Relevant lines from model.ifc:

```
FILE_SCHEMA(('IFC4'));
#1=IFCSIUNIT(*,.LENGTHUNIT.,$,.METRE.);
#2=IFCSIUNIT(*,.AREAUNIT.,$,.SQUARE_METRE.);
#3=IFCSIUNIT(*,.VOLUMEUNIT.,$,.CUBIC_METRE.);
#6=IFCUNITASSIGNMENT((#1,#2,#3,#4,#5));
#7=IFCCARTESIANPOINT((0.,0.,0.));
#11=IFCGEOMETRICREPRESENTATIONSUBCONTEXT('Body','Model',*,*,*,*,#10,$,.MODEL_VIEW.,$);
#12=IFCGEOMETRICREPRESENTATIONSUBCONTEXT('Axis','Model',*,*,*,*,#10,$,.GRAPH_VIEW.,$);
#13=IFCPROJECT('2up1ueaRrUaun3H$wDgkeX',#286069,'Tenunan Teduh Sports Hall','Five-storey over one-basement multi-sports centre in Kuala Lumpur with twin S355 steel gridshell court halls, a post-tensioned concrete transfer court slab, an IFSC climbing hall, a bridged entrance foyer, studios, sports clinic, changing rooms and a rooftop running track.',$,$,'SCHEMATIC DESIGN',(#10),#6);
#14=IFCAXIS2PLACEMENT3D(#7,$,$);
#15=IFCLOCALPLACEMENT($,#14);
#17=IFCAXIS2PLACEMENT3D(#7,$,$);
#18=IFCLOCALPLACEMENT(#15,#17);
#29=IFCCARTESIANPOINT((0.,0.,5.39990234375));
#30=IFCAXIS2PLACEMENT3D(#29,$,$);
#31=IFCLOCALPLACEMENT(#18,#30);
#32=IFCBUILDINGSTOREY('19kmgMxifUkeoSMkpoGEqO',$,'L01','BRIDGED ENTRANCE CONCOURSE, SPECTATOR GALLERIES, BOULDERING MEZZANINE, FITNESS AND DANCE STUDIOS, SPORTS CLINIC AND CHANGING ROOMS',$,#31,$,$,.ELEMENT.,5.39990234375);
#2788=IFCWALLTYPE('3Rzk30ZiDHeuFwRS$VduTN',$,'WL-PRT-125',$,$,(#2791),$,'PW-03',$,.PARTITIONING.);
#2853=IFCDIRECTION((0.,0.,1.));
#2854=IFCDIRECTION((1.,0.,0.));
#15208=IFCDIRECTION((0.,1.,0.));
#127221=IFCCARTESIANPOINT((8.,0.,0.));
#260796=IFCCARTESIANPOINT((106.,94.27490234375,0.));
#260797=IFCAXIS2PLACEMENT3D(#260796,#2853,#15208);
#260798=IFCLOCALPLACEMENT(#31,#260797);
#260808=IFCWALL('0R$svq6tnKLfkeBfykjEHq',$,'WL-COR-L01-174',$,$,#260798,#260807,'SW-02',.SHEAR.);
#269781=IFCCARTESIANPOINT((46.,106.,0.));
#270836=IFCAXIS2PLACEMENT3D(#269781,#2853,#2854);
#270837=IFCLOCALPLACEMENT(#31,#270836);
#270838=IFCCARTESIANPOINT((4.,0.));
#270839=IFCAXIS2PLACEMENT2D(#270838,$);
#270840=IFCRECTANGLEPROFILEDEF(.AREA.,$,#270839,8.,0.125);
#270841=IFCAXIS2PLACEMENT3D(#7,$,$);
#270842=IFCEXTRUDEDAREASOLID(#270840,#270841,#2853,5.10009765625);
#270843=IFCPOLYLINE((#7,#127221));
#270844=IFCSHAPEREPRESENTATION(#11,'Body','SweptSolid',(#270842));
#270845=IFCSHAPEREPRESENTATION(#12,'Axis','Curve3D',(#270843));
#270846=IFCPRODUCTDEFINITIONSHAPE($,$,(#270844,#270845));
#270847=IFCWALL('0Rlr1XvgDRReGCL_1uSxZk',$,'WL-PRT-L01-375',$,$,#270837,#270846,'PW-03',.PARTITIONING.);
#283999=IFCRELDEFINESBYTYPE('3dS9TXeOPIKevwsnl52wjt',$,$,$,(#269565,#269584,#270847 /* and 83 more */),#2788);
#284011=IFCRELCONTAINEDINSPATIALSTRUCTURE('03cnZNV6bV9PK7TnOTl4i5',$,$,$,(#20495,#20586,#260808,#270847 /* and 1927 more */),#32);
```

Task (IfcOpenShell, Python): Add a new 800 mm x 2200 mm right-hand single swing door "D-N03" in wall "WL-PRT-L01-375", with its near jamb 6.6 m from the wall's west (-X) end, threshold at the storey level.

```python
import numpy as np
import ifcopenshell
import ifcopenshell.api.feature
import ifcopenshell.api.geometry
import ifcopenshell.api.root
import ifcopenshell.api.spatial
import ifcopenshell.geom
import ifcopenshell.util.element
import ifcopenshell.util.placement
import ifcopenshell.util.representation
import ifcopenshell.util.shape
import ifcopenshell.util.unit

model = ifcopenshell.open("model.ifc")
unit_scale = ifcopenshell.util.unit.calculate_unit_scale(model)
settings = ifcopenshell.geom.settings()


def volume(element):
    """Net volume in cubic metres, openings subtracted."""
    shape = ifcopenshell.geom.create_shape(settings, element)
    return ifcopenshell.util.shape.get_volume(shape.geometry)


wall = model.by_guid("0Rlr1XvgDRReGCL_1uSxZk")
storey = ifcopenshell.util.element.get_container(wall, ifc_class="IfcBuildingStorey")
context = ifcopenshell.util.representation.get_context(model, "Model", "Body", "MODEL_VIEW")
before = volume(wall)

width, height, from_end, sill = 0.8, 2.2, 6.6, 0.0  # metres

# The wall runs along its own X axis, and the end named is its -X end.
wall_shape = ifcopenshell.geom.create_shape(settings, wall)
x, y, z = ifcopenshell.util.shape.get_vertices(wall_shape.geometry).T
start = x.min() + from_end
face, thickness = float(y.min()), float(y.max() - y.min())
wall_matrix = ifcopenshell.util.placement.get_local_placement(wall.ObjectPlacement)
level = ifcopenshell.util.placement.get_local_placement(storey.ObjectPlacement)[2, 3]


def in_wall(x, y):
    """Placement at x, y metres in the wall's axes, at sill height."""
    matrix = wall_matrix.copy()
    matrix[:, 3] = wall_matrix @ np.array([x / unit_scale, y / unit_scale, 0.0, 1.0])
    matrix[2, 3] = level + sill / unit_scale
    return matrix


# Opening: a box that overshoots both wall faces by 50 mm.
opening = ifcopenshell.api.root.create_entity(model, ifc_class="IfcOpeningElement", predefined_type="OPENING")
box = ifcopenshell.api.geometry.add_wall_representation(
    model, context=context, length=width, height=height, thickness=thickness + 0.1
)
ifcopenshell.api.geometry.assign_representation(model, product=opening, representation=box)
ifcopenshell.api.geometry.edit_object_placement(model, product=opening, matrix=in_wall(start, face - 0.05), is_si=False)
ifcopenshell.api.feature.add_feature(model, feature=opening, element=wall)

door = ifcopenshell.api.root.create_entity(model, ifc_class="IfcDoor", name="D-N03", predefined_type="DOOR")
door.OverallWidth, door.OverallHeight = width / unit_scale, height / unit_scale
door.OperationType = "SINGLE_SWING_RIGHT"
body = ifcopenshell.api.geometry.add_door_representation(
    model,
    context=context,
    overall_width=door.OverallWidth,
    overall_height=door.OverallHeight,
    operation_type="SINGLE_SWING_RIGHT",
    lining_properties={"LiningDepth": thickness / unit_scale, "ThresholdDepth": thickness / unit_scale},
)
ifcopenshell.api.geometry.assign_representation(model, product=door, representation=body)
ifcopenshell.api.spatial.assign_container(model, products=[door], relating_structure=storey)
ifcopenshell.api.feature.add_filling(model, opening=opening, element=door)

# The lining spans the wall, so the door starts at the wall face.
ifcopenshell.api.geometry.edit_object_placement(model, product=door, matrix=in_wall(start, face), is_si=False)

after = volume(wall)

print(f"wall volume {before:.3f} -> {after:.3f} m3")

model.write("model_edited.ifc")
```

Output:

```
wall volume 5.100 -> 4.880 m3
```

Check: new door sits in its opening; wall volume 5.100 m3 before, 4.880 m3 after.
